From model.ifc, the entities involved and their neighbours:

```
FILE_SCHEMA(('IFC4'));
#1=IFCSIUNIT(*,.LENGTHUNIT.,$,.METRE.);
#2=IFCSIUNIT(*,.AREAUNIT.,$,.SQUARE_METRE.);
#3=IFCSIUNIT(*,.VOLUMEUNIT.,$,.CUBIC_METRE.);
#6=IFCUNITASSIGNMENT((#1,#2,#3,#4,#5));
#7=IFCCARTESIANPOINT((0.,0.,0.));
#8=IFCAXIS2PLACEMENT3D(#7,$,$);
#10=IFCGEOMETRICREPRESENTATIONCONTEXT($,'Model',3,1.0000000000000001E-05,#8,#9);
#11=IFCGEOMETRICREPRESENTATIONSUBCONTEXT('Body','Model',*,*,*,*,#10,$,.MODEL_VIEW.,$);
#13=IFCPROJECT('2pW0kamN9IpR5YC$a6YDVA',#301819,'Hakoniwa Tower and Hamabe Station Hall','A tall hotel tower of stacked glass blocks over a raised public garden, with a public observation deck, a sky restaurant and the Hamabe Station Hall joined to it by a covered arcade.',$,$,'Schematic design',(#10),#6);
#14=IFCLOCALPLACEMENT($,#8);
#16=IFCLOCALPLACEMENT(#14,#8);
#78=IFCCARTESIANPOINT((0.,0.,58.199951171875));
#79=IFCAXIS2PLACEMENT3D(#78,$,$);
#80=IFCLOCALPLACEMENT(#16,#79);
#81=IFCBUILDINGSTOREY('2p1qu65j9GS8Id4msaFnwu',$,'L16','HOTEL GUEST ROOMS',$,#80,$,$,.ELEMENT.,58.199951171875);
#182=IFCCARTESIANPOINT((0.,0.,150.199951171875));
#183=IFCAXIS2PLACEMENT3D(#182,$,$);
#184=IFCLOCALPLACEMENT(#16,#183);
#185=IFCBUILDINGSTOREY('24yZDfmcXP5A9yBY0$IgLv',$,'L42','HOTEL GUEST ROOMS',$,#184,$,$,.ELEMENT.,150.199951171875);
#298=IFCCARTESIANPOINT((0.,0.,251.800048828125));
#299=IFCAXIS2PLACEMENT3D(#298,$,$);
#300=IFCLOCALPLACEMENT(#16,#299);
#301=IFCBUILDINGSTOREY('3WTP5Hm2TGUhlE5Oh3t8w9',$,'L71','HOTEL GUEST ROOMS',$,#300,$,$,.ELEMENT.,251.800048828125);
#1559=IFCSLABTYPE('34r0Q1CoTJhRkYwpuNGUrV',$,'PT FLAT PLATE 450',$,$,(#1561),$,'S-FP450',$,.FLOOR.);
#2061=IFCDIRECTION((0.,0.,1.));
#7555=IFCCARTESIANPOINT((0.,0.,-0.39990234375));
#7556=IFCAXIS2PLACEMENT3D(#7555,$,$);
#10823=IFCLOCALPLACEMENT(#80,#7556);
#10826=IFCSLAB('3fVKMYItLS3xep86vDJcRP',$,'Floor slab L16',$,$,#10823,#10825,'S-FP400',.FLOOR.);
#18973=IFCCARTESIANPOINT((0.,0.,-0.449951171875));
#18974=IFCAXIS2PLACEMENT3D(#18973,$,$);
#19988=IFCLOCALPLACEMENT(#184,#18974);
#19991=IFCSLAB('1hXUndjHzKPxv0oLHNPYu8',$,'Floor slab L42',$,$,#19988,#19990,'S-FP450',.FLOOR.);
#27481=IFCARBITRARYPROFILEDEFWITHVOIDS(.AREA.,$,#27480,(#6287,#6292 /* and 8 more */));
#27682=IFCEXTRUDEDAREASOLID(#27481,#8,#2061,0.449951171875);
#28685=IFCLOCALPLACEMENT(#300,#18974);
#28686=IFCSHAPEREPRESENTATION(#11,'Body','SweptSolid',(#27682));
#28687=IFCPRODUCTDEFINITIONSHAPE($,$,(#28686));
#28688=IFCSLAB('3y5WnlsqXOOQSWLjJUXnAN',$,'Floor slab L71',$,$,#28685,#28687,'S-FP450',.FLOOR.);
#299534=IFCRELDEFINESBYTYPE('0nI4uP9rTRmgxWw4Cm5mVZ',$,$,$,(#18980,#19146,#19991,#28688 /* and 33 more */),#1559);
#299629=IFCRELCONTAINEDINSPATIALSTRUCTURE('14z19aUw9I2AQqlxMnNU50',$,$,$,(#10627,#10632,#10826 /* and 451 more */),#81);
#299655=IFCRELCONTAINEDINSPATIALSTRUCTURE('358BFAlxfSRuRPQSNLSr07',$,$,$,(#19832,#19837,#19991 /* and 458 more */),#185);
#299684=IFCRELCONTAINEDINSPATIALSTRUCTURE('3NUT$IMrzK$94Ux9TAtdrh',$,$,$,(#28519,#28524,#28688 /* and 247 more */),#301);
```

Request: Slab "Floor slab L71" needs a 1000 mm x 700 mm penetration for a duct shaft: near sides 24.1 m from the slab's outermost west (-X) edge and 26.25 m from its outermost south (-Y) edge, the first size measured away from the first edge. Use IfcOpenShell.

```python
import numpy as np
import ifcopenshell
import ifcopenshell.api.feature
import ifcopenshell.api.geometry
import ifcopenshell.api.root
import ifcopenshell.geom
import ifcopenshell.util.placement
import ifcopenshell.util.representation
import ifcopenshell.util.shape
import ifcopenshell.util.unit

model = ifcopenshell.open("model.ifc")
unit_scale = ifcopenshell.util.unit.calculate_unit_scale(model)
settings = ifcopenshell.geom.settings()


def volume(element):
    """Net volume in cubic metres, openings subtracted."""
    shape = ifcopenshell.geom.create_shape(settings, element)
    return ifcopenshell.util.shape.get_volume(shape.geometry)


slab = model.by_guid("3y5WnlsqXOOQSWLjJUXnAN")
before = volume(slab)

# Extent in the slab's own axes, in metres. The edges named are its -X and -Y sides.
slab_shape = ifcopenshell.geom.create_shape(settings, slab)
vertices = ifcopenshell.util.shape.get_vertices(slab_shape.geometry)
x_min, y_min, bottom = vertices.min(axis=0)
top = vertices[:, 2].max()

opening = ifcopenshell.api.root.create_entity(model, ifc_class="IfcOpeningElement", name="Duct shaft opening", predefined_type="OPENING")
context = ifcopenshell.util.representation.get_context(model, "Model", "Body", "MODEL_VIEW")
width, depth = 1, 0.7
outline = [(0.0, 0.0), (width, 0.0), (width, depth), (0.0, depth), (0.0, 0.0)]
# Overshoot both faces by 50 mm so the cut is clean.
shape = ifcopenshell.api.geometry.add_slab_representation(
    model, context=context, depth=top - bottom + 0.1, polyline=outline
)
ifcopenshell.api.geometry.assign_representation(model, product=opening, representation=shape)

matrix = ifcopenshell.util.placement.get_local_placement(slab.ObjectPlacement)
matrix[:, 3] = matrix @ np.append(np.array([x_min + 24.1, y_min + 26.25, bottom - 0.05]) / unit_scale, 1.0)
ifcopenshell.api.geometry.edit_object_placement(model, product=opening, matrix=matrix, is_si=False)
ifcopenshell.api.feature.add_feature(model, feature=opening, element=slab)

after = volume(slab)

print(f"slab volume {before:.3f} -> {after:.3f} m3")

model.write("model-out.ifc")
```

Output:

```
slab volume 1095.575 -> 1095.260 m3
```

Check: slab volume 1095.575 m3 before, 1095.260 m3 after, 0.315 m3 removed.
